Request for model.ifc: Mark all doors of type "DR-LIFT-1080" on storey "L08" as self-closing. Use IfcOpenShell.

First a look at what the model holds.

```python
import ifcopenshell
import ifcopenshell.util.element

model = ifcopenshell.open("model.ifc")
print(model.schema)
storey = next(s for s in model.by_type("IfcBuildingStorey") if s.Name == "L08")
doors = [e for e in ifcopenshell.util.element.get_decomposition(storey) if e.is_a("IfcDoor")]
seen = {}
for e in doors:
    element_type = ifcopenshell.util.element.get_type(e)
    key = (element_type.Name if element_type != e and element_type else None, ifcopenshell.util.element.get_pset(e, "Pset_DoorCommon", "SelfClosing"))
    seen[key] = seen.get(key, 0) + 1
for (name, value), count in sorted(seen.items(), key=str):
    print(count, "x", name, "|", value)
```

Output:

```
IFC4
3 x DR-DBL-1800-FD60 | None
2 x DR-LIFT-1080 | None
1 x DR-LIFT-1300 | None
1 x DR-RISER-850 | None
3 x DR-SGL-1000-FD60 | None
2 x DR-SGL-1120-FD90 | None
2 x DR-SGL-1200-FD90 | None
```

```python
import ifcopenshell
import ifcopenshell.api.pset
import ifcopenshell.util.element

model = ifcopenshell.open("model.ifc")

storey = next(s for s in model.by_type("IfcBuildingStorey") if s.Name == "L08")
doors = [e for e in ifcopenshell.util.element.get_decomposition(storey) if e.is_a("IfcDoor")]

count = 0
for e in doors:
    element_type = ifcopenshell.util.element.get_type(e)
    if element_type in (None, e) or element_type.Name != "DR-LIFT-1080":
        continue
    # add_pset returns the element's existing set when there is one.
    pset = ifcopenshell.api.pset.add_pset(model, product=e, name="Pset_DoorCommon")
    ifcopenshell.api.pset.edit_pset(model, pset=pset, properties={"SelfClosing": True})
    count += 1

print(count, "doors updated")

model.write("model-out.ifc")
```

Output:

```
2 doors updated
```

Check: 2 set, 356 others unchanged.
